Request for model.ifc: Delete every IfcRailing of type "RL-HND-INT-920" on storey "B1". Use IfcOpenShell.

First a look at what the model holds.

```python
import ifcopenshell
import ifcopenshell.util.element

model = ifcopenshell.open("model.ifc")
print(model.schema)
storey = next(s for s in model.by_type("IfcBuildingStorey") if s.Name == "B1")
railings = [e for e in ifcopenshell.util.element.get_decomposition(storey) if e.is_a("IfcRailing")]
seen = {}
for e in railings:
    element_type = ifcopenshell.util.element.get_type(e)
    name = element_type.Name if element_type not in (None, e) else None
    seen[name] = seen.get(name, 0) + 1
for name, count in sorted(seen.items(), key=str):
    print(count, "x", name)
```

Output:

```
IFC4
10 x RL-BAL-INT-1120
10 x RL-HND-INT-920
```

```python
import ifcopenshell
import ifcopenshell.api.root
import ifcopenshell.util.element

model = ifcopenshell.open("model.ifc")

storey = next(s for s in model.by_type("IfcBuildingStorey") if s.Name == "B1")
railings = [e for e in ifcopenshell.util.element.get_decomposition(storey) if e.is_a("IfcRailing")]
targets = [e for e in railings if (t := ifcopenshell.util.element.get_type(e)) not in (None, e) and t.Name == "RL-HND-INT-920"]

for e in targets:
    ifcopenshell.api.root.remove_product(model, product=e)
print(len(targets), "removed")

model.write("model_updated.ifc")
```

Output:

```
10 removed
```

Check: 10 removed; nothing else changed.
